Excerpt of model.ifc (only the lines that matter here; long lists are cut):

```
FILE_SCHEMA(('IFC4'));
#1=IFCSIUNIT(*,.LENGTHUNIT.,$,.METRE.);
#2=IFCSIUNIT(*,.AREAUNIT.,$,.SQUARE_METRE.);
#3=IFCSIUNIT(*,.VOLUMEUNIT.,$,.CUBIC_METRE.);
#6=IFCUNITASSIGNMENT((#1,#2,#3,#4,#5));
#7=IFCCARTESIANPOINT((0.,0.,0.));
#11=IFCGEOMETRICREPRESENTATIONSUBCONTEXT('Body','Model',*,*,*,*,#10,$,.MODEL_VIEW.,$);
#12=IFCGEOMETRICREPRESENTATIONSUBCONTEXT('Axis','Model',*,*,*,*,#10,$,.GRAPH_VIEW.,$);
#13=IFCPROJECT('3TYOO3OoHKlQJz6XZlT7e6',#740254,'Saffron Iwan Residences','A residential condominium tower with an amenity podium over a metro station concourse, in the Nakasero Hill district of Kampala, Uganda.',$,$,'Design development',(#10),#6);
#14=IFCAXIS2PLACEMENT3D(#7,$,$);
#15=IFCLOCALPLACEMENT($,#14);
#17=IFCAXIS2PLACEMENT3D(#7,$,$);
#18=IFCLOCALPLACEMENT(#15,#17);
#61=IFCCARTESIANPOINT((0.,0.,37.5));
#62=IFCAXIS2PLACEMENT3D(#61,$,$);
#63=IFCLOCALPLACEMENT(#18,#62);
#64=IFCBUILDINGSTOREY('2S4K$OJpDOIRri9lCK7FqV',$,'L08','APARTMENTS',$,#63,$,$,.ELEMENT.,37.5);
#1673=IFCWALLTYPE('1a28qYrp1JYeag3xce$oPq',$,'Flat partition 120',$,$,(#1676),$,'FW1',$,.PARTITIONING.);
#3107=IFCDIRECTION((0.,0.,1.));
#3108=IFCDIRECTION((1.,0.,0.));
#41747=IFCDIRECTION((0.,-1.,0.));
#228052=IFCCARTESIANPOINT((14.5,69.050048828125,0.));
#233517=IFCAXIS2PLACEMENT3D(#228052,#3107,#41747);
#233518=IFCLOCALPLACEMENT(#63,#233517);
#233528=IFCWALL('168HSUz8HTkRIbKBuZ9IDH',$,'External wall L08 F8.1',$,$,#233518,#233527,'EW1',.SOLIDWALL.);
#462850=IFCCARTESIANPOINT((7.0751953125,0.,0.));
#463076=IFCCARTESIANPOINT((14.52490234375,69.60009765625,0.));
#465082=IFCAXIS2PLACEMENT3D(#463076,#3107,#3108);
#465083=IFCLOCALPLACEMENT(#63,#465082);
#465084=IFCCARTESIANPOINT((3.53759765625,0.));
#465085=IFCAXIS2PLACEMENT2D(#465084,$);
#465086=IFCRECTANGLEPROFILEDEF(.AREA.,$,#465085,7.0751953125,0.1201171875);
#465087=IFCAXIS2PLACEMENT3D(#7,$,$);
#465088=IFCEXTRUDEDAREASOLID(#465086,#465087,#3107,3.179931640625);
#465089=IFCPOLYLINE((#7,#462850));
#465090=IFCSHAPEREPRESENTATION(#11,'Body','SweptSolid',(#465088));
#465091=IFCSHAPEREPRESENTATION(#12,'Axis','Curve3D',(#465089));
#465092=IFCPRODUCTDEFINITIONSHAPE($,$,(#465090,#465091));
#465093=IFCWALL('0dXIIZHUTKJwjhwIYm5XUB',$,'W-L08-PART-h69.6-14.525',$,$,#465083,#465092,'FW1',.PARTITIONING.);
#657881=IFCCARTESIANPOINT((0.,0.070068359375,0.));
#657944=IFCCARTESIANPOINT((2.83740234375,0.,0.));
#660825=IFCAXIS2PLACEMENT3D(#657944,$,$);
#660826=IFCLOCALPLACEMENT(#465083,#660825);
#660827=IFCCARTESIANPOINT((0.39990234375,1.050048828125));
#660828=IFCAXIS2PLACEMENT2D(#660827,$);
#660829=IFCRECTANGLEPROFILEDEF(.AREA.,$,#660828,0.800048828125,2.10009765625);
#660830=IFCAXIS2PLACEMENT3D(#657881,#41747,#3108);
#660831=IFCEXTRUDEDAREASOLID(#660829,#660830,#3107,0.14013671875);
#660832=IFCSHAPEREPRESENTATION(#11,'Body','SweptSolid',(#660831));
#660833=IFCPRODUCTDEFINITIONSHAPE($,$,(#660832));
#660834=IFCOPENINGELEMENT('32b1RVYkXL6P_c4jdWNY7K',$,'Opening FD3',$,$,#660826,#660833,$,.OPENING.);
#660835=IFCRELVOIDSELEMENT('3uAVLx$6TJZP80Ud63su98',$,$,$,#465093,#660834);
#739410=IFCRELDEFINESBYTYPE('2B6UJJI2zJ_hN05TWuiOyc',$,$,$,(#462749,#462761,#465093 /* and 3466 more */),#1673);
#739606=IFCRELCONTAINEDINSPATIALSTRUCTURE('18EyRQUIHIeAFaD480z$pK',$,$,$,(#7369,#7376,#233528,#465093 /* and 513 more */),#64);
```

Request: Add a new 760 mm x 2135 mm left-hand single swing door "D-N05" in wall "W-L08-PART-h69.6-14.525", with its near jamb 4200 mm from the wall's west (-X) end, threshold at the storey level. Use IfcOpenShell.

```python
import numpy as np
import ifcopenshell
import ifcopenshell.api.feature
import ifcopenshell.api.geometry
import ifcopenshell.api.root
import ifcopenshell.api.spatial
import ifcopenshell.geom
import ifcopenshell.util.element
import ifcopenshell.util.placement
import ifcopenshell.util.representation
import ifcopenshell.util.shape
import ifcopenshell.util.unit

model = ifcopenshell.open("model.ifc")
unit_scale = ifcopenshell.util.unit.calculate_unit_scale(model)
settings = ifcopenshell.geom.settings()


def volume(element):
    """Net volume in cubic metres, openings subtracted."""
    shape = ifcopenshell.geom.create_shape(settings, element)
    return ifcopenshell.util.shape.get_volume(shape.geometry)


wall = model.by_guid("0dXIIZHUTKJwjhwIYm5XUB")
storey = ifcopenshell.util.element.get_container(wall, ifc_class="IfcBuildingStorey")
context = ifcopenshell.util.representation.get_context(model, "Model", "Body", "MODEL_VIEW")
before = volume(wall)

width, height, from_end, sill = 0.76, 2.135, 4.2, 0.0  # metres

# The wall runs along its own X axis, and the end named is its -X end.
wall_shape = ifcopenshell.geom.create_shape(settings, wall)
x, y, z = ifcopenshell.util.shape.get_vertices(wall_shape.geometry).T
start = x.min() + from_end
face, thickness = float(y.min()), float(y.max() - y.min())
wall_matrix = ifcopenshell.util.placement.get_local_placement(wall.ObjectPlacement)
level = ifcopenshell.util.placement.get_local_placement(storey.ObjectPlacement)[2, 3]


def in_wall(x, y):
    """Placement at x, y metres in the wall's axes, at sill height."""
    matrix = wall_matrix.copy()
    matrix[:, 3] = wall_matrix @ np.array([x / unit_scale, y / unit_scale, 0.0, 1.0])
    matrix[2, 3] = level + sill / unit_scale
    return matrix


# Opening: a box that overshoots both wall faces by 50 mm.
opening = ifcopenshell.api.root.create_entity(model, ifc_class="IfcOpeningElement", predefined_type="OPENING")
box = ifcopenshell.api.geometry.add_wall_representation(
    model, context=context, length=width, height=height, thickness=thickness + 0.1
)
ifcopenshell.api.geometry.assign_representation(model, product=opening, representation=box)
ifcopenshell.api.geometry.edit_object_placement(model, product=opening, matrix=in_wall(start, face - 0.05), is_si=False)
ifcopenshell.api.feature.add_feature(model, feature=opening, element=wall)

door = ifcopenshell.api.root.create_entity(model, ifc_class="IfcDoor", name="D-N05", predefined_type="DOOR")
door.OverallWidth, door.OverallHeight = width / unit_scale, height / unit_scale
door.OperationType = "SINGLE_SWING_LEFT"
body = ifcopenshell.api.geometry.add_door_representation(
    model,
    context=context,
    overall_width=door.OverallWidth,
    overall_height=door.OverallHeight,
    operation_type="SINGLE_SWING_LEFT",
    lining_properties={"LiningDepth": thickness / unit_scale, "ThresholdDepth": thickness / unit_scale},
)
ifcopenshell.api.geometry.assign_representation(model, product=door, representation=body)
ifcopenshell.api.spatial.assign_container(model, products=[door], relating_structure=storey)
ifcopenshell.api.feature.add_filling(model, opening=opening, element=door)

# The lining spans the wall, so the door starts at the wall face.
ifcopenshell.api.geometry.edit_object_placement(model, product=door, matrix=in_wall(start, face), is_si=False)

after = volume(wall)

print(f"wall volume {before:.3f} -> {after:.3f} m3")

model.write("model-out.ifc")
```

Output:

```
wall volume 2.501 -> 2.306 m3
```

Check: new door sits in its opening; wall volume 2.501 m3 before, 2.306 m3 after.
